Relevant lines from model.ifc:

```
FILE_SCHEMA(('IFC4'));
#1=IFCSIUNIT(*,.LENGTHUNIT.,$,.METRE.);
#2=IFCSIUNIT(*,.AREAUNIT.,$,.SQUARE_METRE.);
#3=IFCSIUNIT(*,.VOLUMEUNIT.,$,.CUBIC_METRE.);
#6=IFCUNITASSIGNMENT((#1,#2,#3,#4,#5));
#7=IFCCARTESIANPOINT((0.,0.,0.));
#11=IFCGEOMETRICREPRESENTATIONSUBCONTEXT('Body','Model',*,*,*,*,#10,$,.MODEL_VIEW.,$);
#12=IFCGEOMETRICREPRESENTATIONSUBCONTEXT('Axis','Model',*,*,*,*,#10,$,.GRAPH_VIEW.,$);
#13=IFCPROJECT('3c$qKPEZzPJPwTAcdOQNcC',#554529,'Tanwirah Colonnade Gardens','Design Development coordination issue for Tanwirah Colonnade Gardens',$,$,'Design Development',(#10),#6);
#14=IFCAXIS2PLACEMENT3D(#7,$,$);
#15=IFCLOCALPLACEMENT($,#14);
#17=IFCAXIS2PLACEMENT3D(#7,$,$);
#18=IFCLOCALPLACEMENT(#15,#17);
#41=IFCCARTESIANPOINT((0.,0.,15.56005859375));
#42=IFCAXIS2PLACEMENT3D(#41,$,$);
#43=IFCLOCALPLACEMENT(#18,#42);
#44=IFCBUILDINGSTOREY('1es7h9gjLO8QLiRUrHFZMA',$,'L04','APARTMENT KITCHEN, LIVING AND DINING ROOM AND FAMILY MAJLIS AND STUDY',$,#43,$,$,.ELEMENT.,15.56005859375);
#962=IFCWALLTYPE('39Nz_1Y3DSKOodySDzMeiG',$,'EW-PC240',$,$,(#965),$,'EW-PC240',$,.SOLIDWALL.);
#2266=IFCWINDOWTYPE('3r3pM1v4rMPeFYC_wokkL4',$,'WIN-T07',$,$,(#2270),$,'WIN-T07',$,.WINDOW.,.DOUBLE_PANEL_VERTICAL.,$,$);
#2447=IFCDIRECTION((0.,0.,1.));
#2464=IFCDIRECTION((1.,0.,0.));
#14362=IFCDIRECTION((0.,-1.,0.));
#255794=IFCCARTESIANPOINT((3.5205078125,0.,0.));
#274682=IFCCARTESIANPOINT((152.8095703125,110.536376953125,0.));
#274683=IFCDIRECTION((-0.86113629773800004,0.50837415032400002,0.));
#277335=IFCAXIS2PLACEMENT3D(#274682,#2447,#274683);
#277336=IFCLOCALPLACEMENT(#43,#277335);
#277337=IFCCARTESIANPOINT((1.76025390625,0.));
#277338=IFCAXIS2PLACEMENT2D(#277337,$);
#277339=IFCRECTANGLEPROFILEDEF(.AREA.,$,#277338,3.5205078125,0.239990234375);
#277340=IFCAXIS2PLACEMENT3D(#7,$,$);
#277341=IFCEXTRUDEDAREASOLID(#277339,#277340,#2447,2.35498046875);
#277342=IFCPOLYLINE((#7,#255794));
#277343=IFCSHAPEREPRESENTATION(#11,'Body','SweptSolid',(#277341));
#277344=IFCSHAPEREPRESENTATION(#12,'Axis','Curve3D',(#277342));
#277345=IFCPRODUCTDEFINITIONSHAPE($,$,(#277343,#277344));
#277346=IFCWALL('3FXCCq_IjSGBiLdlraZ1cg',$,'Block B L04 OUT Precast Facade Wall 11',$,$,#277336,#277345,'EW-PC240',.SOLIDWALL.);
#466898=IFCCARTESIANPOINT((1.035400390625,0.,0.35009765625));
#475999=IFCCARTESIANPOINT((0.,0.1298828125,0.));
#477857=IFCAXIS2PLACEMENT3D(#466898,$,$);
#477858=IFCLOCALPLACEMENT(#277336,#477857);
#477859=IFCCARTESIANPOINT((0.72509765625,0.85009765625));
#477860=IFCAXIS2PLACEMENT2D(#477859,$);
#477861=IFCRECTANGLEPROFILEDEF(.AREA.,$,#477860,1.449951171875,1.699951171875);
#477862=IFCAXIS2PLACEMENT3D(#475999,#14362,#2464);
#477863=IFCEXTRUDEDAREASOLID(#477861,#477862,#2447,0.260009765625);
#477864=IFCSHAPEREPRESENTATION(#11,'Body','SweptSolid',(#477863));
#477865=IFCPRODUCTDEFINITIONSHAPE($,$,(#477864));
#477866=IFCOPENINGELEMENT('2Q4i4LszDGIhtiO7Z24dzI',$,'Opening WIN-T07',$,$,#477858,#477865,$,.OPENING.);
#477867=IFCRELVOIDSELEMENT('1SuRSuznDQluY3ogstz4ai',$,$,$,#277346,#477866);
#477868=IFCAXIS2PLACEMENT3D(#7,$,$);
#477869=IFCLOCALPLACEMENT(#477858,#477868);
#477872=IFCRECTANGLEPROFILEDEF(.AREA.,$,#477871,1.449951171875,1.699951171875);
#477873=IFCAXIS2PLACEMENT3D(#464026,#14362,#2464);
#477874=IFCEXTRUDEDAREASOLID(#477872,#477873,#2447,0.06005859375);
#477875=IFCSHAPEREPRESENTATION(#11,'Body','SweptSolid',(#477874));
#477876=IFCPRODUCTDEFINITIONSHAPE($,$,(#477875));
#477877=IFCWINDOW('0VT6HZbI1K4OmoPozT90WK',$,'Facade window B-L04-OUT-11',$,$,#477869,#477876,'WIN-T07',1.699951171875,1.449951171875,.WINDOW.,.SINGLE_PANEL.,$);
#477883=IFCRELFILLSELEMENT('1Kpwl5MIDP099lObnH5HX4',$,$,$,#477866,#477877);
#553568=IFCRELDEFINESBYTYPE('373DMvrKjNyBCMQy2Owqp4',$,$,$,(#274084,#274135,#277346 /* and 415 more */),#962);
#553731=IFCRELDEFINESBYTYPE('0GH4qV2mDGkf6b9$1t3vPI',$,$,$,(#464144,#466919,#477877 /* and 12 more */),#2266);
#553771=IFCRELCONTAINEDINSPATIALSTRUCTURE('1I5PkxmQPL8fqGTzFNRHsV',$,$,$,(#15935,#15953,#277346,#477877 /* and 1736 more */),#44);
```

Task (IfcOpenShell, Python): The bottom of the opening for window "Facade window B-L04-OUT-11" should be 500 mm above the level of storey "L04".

```python
import numpy as np
import ifcopenshell
import ifcopenshell.api.geometry
import ifcopenshell.geom
import ifcopenshell.util.element
import ifcopenshell.util.placement
import ifcopenshell.util.shape
import ifcopenshell.util.unit

model = ifcopenshell.open("model.ifc")
unit_scale = ifcopenshell.util.unit.calculate_unit_scale(model)

window = model.by_guid("0VT6HZbI1K4OmoPozT90WK")
opening = window.FillsVoids[0].RelatingOpeningElement
storey = ifcopenshell.util.element.get_container(window, ifc_class="IfcBuildingStorey")
level = ifcopenshell.util.placement.get_local_placement(storey.ObjectPlacement)[2, 3]

# The opening's origin need not be at the sill, so measure its lowest point.
shape = ifcopenshell.geom.create_shape(ifcopenshell.geom.settings(), opening)
bottom = ifcopenshell.util.shape.get_shape_bottom_elevation(shape, shape.geometry) / unit_scale
dz = level + 0.5 - bottom

shift = np.array([0.0, 0.0, dz])
# The window is placed relative to its opening, so it follows when the opening moves.
matrix = ifcopenshell.util.placement.get_local_placement(opening.ObjectPlacement)
matrix[:3, 3] += shift
ifcopenshell.api.geometry.edit_object_placement(
    model, product=opening, matrix=matrix, is_si=False, should_transform_children=True
)

print(f"moved by {dz * unit_scale:+.3f} m")

model.write("model_v2.ifc")
```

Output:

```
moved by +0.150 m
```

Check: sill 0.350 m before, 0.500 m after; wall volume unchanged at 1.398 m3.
